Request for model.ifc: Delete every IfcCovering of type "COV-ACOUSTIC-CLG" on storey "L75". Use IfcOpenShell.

First a look at what the model holds.

```python
import ifcopenshell
import ifcopenshell.util.element

model = ifcopenshell.open("model.ifc")
print(model.schema)
storey = next(s for s in model.by_type("IfcBuildingStorey") if s.Name == "L75")
coverings = [e for e in ifcopenshell.util.element.get_decomposition(storey) if e.is_a("IfcCovering")]
seen = {}
for e in coverings:
    element_type = ifcopenshell.util.element.get_type(e)
    name = element_type.Name if element_type not in (None, e) else None
    seen[name] = seen.get(name, 0) + 1
for name, count in sorted(seen.items(), key=str):
    print(count, "x", name)
```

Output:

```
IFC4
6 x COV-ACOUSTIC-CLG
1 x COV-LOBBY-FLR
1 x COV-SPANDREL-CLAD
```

```python
import ifcopenshell
import ifcopenshell.api.root
import ifcopenshell.util.element

model = ifcopenshell.open("model.ifc")

storey = next(s for s in model.by_type("IfcBuildingStorey") if s.Name == "L75")
coverings = [e for e in ifcopenshell.util.element.get_decomposition(storey) if e.is_a("IfcCovering")]
targets = [e for e in coverings if (t := ifcopenshell.util.element.get_type(e)) not in (None, e) and t.Name == "COV-ACOUSTIC-CLG"]

for e in targets:
    ifcopenshell.api.root.remove_product(model, product=e)
print(len(targets), "removed")

model.write("model_v2.ifc")
```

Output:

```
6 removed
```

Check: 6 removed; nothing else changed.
